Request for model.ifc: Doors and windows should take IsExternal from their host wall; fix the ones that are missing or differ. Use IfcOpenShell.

First a look at what the model holds.

```python
import ifcopenshell
import ifcopenshell.util.element

model = ifcopenshell.open("model.ifc")
print(model.schema)
seen = {}
for e in model.by_type("IfcDoor") + model.by_type("IfcWindow"):
    if not e.FillsVoids:
        continue
    host = e.FillsVoids[0].RelatingOpeningElement.VoidsElements[0].RelatingBuildingElement
    own = ifcopenshell.util.element.get_pset(e, f"Pset_{e.is_a()[3:].removesuffix('StandardCase')}Common", "IsExternal")
    wall = ifcopenshell.util.element.get_pset(host, "Pset_WallCommon", "IsExternal")
    seen[e.is_a(), own, wall] = seen.get((e.is_a(), own, wall), 0) + 1
for (cls, own, wall), count in sorted(seen.items(), key=str):
    print(count, cls, "IsExternal:", own, "| host wall:", wall)
```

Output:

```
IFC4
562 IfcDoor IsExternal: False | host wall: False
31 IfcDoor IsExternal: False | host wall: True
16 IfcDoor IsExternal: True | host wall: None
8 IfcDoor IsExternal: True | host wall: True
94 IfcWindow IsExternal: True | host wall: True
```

```python
import ifcopenshell
import ifcopenshell.api.pset
import ifcopenshell.util.element

model = ifcopenshell.open("model.ifc")

count = 0
for ifc_class, pset_name in (("IfcDoor", "Pset_DoorCommon"), ("IfcWindow", "Pset_WindowCommon")):
    for e in model.by_type(ifc_class):
        if not e.FillsVoids:
            continue
        host = e.FillsVoids[0].RelatingOpeningElement.VoidsElements[0].RelatingBuildingElement
        external = ifcopenshell.util.element.get_pset(host, "Pset_WallCommon", "IsExternal")
        if external is None or ifcopenshell.util.element.get_pset(e, pset_name, "IsExternal") == external:
            continue
        pset = ifcopenshell.api.pset.add_pset(model, product=e, name=pset_name)
        ifcopenshell.api.pset.edit_pset(model, pset=pset, properties={"IsExternal": external})
        count += 1

print(count, "updated")

model.write("model_updated.ifc")
```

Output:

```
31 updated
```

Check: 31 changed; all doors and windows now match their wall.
